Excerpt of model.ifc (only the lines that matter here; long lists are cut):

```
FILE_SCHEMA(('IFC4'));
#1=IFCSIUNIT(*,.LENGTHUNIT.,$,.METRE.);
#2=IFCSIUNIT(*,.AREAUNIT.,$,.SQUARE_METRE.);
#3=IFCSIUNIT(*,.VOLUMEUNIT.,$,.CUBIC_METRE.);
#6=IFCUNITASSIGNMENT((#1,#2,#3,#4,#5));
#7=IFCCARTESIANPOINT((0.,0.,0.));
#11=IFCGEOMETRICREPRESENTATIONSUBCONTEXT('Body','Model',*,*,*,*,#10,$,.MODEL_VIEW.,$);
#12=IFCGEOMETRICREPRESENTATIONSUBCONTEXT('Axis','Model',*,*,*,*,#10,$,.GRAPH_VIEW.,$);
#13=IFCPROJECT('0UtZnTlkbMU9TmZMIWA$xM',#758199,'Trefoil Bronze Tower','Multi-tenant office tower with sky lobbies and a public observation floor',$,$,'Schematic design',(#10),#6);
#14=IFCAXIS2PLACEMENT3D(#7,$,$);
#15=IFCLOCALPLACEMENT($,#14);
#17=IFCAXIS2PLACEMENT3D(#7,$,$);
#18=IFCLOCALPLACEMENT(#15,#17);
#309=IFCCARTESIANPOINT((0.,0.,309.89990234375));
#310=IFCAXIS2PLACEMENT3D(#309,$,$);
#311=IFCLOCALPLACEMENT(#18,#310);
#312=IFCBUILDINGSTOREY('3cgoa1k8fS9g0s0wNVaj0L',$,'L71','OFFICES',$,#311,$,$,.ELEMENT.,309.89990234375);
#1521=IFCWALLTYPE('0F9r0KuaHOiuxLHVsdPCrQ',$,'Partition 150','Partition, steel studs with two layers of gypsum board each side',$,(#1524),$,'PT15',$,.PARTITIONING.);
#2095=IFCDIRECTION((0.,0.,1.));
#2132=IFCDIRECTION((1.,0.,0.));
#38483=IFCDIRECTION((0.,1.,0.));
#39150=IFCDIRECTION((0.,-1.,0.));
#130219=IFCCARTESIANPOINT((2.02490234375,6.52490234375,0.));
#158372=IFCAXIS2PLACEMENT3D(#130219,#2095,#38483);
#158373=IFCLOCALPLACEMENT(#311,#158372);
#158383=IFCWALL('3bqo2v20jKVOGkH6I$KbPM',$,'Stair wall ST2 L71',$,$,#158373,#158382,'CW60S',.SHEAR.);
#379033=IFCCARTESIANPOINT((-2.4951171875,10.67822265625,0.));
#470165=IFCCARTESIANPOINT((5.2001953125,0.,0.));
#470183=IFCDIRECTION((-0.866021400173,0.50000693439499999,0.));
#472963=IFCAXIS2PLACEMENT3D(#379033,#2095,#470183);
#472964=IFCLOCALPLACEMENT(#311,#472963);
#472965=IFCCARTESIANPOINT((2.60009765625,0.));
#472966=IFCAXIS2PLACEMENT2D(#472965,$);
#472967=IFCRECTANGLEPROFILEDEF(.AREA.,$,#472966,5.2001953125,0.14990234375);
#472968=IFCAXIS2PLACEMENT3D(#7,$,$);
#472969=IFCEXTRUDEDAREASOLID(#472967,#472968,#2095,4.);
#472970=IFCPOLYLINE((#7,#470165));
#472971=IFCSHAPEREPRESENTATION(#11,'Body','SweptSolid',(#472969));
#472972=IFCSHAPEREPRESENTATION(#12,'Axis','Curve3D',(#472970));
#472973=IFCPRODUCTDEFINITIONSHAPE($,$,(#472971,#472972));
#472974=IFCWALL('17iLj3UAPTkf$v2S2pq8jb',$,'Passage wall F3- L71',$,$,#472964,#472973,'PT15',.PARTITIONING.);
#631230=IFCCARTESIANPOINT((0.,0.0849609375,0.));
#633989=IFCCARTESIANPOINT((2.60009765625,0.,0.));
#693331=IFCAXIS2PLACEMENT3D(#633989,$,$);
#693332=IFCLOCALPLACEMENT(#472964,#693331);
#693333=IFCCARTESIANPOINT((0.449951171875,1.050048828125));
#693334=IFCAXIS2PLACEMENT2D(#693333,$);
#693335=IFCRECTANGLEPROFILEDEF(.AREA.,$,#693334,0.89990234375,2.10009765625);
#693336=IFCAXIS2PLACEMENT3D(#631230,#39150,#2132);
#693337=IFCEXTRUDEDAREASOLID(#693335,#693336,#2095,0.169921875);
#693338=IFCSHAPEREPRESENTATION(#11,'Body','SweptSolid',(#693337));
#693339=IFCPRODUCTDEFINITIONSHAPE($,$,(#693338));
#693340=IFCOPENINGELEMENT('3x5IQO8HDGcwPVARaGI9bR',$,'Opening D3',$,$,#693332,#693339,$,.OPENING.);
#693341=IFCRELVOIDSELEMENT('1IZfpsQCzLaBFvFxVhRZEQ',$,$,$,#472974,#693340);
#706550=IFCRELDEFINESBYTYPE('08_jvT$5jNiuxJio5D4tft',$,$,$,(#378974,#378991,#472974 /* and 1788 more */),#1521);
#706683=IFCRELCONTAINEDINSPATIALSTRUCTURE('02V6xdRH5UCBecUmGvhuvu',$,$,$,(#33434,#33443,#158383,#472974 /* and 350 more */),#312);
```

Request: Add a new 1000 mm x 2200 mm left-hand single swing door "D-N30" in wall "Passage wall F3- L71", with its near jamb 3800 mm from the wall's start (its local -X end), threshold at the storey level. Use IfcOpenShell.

```python
import numpy as np
import ifcopenshell
import ifcopenshell.api.feature
import ifcopenshell.api.geometry
import ifcopenshell.api.root
import ifcopenshell.api.spatial
import ifcopenshell.geom
import ifcopenshell.util.element
import ifcopenshell.util.placement
import ifcopenshell.util.representation
import ifcopenshell.util.shape
import ifcopenshell.util.unit

model = ifcopenshell.open("model.ifc")
unit_scale = ifcopenshell.util.unit.calculate_unit_scale(model)
settings = ifcopenshell.geom.settings()


def volume(element):
    """Net volume in cubic metres, openings subtracted."""
    shape = ifcopenshell.geom.create_shape(settings, element)
    return ifcopenshell.util.shape.get_volume(shape.geometry)


wall = model.by_guid("17iLj3UAPTkf$v2S2pq8jb")
storey = ifcopenshell.util.element.get_container(wall, ifc_class="IfcBuildingStorey")
context = ifcopenshell.util.representation.get_context(model, "Model", "Body", "MODEL_VIEW")
before = volume(wall)

width, height, from_end, sill = 1, 2.2, 3.8, 0.0  # metres

# The wall runs along its own X axis, and the end named is its -X end.
wall_shape = ifcopenshell.geom.create_shape(settings, wall)
x, y, z = ifcopenshell.util.shape.get_vertices(wall_shape.geometry).T
start = x.min() + from_end
face, thickness = float(y.min()), float(y.max() - y.min())
wall_matrix = ifcopenshell.util.placement.get_local_placement(wall.ObjectPlacement)
level = ifcopenshell.util.placement.get_local_placement(storey.ObjectPlacement)[2, 3]


def in_wall(x, y):
    """Placement at x, y metres in the wall's axes, at sill height."""
    matrix = wall_matrix.copy()
    matrix[:, 3] = wall_matrix @ np.array([x / unit_scale, y / unit_scale, 0.0, 1.0])
    matrix[2, 3] = level + sill / unit_scale
    return matrix


# Opening: a box that overshoots both wall faces by 50 mm.
opening = ifcopenshell.api.root.create_entity(model, ifc_class="IfcOpeningElement", predefined_type="OPENING")
box = ifcopenshell.api.geometry.add_wall_representation(
    model, context=context, length=width, height=height, thickness=thickness + 0.1
)
ifcopenshell.api.geometry.assign_representation(model, product=opening, representation=box)
ifcopenshell.api.geometry.edit_object_placement(model, product=opening, matrix=in_wall(start, face - 0.05), is_si=False)
ifcopenshell.api.feature.add_feature(model, feature=opening, element=wall)

door = ifcopenshell.api.root.create_entity(model, ifc_class="IfcDoor", name="D-N30", predefined_type="DOOR")
door.OverallWidth, door.OverallHeight = width / unit_scale, height / unit_scale
door.OperationType = "SINGLE_SWING_LEFT"
body = ifcopenshell.api.geometry.add_door_representation(
    model,
    context=context,
    overall_width=door.OverallWidth,
    overall_height=door.OverallHeight,
    operation_type="SINGLE_SWING_LEFT",
    lining_properties={"LiningDepth": thickness / unit_scale, "ThresholdDepth": thickness / unit_scale},
)
ifcopenshell.api.geometry.assign_representation(model, product=door, representation=body)
ifcopenshell.api.spatial.assign_container(model, products=[door], relating_structure=storey)
ifcopenshell.api.feature.add_filling(model, opening=opening, element=door)

# The lining spans the wall, so the door starts at the wall face.
ifcopenshell.api.geometry.edit_object_placement(model, product=door, matrix=in_wall(start, face), is_si=False)

after = volume(wall)

print(f"wall volume {before:.3f} -> {after:.3f} m3")

model.write("model-out.ifc")
```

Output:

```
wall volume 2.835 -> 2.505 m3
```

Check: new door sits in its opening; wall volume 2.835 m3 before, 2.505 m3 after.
